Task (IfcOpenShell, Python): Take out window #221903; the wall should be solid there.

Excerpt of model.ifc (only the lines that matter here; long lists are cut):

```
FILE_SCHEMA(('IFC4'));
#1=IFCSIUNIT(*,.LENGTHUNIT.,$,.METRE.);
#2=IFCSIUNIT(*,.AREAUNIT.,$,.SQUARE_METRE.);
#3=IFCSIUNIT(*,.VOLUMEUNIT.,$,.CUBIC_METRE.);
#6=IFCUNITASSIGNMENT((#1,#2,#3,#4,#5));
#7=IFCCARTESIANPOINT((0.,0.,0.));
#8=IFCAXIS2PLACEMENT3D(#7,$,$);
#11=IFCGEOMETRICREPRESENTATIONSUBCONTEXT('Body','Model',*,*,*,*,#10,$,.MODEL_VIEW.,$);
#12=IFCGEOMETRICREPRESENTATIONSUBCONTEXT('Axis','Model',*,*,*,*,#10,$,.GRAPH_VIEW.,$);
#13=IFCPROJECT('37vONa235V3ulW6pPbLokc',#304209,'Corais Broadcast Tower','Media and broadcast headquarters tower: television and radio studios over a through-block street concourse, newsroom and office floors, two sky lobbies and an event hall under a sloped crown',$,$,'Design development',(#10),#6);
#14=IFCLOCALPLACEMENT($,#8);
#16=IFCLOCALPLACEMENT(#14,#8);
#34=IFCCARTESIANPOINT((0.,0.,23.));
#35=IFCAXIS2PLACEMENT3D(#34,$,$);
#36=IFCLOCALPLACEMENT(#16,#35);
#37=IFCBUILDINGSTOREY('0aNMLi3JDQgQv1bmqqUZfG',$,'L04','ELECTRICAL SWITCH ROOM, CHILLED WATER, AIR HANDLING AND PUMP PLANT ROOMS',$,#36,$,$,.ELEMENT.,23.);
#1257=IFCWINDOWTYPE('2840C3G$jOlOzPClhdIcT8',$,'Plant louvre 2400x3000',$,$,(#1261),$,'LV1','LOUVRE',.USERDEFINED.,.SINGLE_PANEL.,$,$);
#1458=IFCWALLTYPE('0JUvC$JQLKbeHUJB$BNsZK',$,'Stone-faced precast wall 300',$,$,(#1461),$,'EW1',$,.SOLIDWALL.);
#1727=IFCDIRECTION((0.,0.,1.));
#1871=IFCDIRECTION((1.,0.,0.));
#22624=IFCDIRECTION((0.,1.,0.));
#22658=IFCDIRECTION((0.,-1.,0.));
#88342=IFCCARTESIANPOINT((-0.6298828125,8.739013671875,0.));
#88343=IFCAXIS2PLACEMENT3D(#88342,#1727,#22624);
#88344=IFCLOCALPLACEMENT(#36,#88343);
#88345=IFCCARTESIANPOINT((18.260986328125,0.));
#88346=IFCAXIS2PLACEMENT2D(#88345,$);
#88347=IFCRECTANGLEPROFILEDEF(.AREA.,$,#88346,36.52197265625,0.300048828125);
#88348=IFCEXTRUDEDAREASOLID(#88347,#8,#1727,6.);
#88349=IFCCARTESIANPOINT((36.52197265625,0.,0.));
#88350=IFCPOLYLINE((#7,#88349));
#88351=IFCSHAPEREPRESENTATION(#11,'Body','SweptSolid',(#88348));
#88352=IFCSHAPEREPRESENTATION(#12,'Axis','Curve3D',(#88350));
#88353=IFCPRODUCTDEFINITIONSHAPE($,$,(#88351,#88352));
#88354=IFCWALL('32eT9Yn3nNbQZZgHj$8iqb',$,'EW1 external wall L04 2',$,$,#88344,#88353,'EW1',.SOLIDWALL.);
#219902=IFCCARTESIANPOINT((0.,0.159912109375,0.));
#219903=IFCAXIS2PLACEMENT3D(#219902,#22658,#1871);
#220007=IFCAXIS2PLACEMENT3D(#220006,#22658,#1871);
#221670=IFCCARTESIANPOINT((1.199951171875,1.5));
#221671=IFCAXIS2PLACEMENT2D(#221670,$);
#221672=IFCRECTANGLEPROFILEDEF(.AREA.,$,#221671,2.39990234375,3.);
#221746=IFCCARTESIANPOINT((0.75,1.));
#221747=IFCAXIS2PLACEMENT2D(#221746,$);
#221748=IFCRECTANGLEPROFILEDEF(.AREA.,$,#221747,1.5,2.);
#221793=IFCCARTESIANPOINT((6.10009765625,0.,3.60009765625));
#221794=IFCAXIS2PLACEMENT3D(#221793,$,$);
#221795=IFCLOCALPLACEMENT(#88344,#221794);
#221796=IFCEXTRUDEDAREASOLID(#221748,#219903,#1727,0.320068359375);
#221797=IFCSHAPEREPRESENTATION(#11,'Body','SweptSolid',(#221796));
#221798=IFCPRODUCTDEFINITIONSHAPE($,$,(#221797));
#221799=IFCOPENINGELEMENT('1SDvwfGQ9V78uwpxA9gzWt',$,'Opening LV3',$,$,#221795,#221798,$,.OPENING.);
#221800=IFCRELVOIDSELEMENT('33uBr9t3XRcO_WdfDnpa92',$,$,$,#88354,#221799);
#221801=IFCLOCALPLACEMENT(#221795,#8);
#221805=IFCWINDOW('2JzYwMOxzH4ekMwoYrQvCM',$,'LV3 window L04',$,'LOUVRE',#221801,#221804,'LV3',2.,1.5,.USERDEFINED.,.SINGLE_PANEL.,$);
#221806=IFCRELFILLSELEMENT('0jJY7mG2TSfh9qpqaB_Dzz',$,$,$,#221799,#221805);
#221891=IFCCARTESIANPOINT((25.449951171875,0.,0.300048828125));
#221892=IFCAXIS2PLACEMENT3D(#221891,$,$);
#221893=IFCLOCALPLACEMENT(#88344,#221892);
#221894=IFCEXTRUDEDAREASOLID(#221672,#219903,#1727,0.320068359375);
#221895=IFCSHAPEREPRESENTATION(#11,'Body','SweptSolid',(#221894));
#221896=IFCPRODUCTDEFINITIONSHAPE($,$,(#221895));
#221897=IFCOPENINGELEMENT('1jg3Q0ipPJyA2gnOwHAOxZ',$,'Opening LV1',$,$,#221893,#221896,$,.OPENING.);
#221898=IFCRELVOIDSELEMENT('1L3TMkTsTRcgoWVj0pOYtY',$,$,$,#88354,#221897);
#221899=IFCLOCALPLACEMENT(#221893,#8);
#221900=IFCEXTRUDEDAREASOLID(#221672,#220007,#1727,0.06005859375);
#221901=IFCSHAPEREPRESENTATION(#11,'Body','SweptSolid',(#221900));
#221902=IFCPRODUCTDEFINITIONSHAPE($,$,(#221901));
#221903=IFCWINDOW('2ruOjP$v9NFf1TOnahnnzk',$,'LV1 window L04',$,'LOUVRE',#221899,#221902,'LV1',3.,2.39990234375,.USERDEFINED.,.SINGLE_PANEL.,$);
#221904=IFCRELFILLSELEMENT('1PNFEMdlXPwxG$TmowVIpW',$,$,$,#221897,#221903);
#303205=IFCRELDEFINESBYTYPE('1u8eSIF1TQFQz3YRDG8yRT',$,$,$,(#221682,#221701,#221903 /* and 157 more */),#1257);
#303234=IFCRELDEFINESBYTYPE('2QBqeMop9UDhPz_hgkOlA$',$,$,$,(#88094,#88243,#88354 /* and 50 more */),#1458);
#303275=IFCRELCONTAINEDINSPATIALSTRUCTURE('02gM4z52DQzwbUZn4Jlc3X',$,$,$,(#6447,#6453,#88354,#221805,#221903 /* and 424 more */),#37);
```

```python
import ifcopenshell
import ifcopenshell.api.feature
import ifcopenshell.api.root
import ifcopenshell.geom
import ifcopenshell.util.shape

model = ifcopenshell.open("model.ifc")
settings = ifcopenshell.geom.settings()


def volume(element):
    """Net volume in cubic metres, openings subtracted."""
    shape = ifcopenshell.geom.create_shape(settings, element)
    return ifcopenshell.util.shape.get_volume(shape.geometry)


window = model.by_guid("2ruOjP$v9NFf1TOnahnnzk")
opening = window.FillsVoids[0].RelatingOpeningElement
wall = opening.VoidsElements[0].RelatingBuildingElement
before = volume(wall)

ifcopenshell.api.root.remove_product(model, product=window)
ifcopenshell.api.feature.remove_feature(model, feature=opening)

after = volume(wall)

print(f"wall volume {before:.3f} -> {after:.3f} m3")

model.write("model_v2.ifc")
```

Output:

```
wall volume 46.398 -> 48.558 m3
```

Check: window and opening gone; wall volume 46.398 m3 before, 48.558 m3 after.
